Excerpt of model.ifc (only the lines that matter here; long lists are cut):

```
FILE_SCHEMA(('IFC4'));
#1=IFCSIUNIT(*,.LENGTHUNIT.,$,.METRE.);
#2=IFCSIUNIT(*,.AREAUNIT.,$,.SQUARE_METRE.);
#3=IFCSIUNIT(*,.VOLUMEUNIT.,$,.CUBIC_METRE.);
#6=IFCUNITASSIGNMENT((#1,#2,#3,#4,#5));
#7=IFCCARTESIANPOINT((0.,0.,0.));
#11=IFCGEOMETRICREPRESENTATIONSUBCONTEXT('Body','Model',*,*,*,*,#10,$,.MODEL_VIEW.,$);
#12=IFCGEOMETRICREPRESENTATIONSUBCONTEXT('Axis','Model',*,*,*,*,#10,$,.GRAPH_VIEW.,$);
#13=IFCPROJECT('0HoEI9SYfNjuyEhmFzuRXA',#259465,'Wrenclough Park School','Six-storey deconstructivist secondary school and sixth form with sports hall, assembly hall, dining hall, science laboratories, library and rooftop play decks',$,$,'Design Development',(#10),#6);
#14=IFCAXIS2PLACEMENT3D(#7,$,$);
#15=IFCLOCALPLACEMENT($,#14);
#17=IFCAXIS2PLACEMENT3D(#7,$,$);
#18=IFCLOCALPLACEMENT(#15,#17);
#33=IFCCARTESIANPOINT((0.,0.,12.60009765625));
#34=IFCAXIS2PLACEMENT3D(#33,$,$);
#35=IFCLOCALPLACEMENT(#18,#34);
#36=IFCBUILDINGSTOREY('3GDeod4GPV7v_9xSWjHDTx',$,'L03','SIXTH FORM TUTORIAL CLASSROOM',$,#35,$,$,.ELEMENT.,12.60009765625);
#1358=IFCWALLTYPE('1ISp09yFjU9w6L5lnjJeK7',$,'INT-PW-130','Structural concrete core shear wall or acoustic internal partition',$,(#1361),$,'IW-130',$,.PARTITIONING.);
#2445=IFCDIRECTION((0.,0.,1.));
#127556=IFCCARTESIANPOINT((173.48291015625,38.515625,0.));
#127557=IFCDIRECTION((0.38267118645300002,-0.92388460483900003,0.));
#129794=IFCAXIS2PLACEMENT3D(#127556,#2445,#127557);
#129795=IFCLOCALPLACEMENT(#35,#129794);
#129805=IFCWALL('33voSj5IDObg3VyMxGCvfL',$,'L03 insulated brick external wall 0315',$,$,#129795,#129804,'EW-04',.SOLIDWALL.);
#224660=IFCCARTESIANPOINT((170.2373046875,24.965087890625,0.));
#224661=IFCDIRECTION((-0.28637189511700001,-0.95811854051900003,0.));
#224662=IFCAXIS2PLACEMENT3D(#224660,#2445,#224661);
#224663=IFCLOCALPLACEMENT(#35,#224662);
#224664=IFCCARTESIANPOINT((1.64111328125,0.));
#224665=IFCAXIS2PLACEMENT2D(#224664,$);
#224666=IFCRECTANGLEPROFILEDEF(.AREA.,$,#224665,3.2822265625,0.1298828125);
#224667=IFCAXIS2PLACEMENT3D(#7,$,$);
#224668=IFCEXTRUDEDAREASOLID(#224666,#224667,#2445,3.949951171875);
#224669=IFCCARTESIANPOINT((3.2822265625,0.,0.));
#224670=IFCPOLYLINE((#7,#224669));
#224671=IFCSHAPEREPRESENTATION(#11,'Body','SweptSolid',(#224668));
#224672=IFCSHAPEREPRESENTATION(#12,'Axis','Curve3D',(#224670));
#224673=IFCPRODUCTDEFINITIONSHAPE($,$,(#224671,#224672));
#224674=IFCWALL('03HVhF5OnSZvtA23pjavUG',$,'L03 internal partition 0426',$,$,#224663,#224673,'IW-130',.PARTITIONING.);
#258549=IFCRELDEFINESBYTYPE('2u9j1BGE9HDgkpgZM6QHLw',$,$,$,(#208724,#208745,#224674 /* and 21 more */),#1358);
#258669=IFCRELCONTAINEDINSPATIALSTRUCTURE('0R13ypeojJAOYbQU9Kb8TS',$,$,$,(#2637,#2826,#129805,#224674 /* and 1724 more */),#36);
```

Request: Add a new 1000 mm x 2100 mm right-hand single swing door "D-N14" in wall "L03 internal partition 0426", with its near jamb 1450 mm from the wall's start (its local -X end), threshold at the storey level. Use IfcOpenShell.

```python
import numpy as np
import ifcopenshell
import ifcopenshell.api.feature
import ifcopenshell.api.geometry
import ifcopenshell.api.root
import ifcopenshell.api.spatial
import ifcopenshell.geom
import ifcopenshell.util.element
import ifcopenshell.util.placement
import ifcopenshell.util.representation
import ifcopenshell.util.shape
import ifcopenshell.util.unit

model = ifcopenshell.open("model.ifc")
unit_scale = ifcopenshell.util.unit.calculate_unit_scale(model)
settings = ifcopenshell.geom.settings()


def volume(element):
    """Net volume in cubic metres, openings subtracted."""
    shape = ifcopenshell.geom.create_shape(settings, element)
    return ifcopenshell.util.shape.get_volume(shape.geometry)


wall = model.by_guid("03HVhF5OnSZvtA23pjavUG")
storey = ifcopenshell.util.element.get_container(wall, ifc_class="IfcBuildingStorey")
context = ifcopenshell.util.representation.get_context(model, "Model", "Body", "MODEL_VIEW")
before = volume(wall)

width, height, from_end, sill = 1, 2.1, 1.45, 0.0  # metres

# The wall runs along its own X axis, and the end named is its -X end.
wall_shape = ifcopenshell.geom.create_shape(settings, wall)
x, y, z = ifcopenshell.util.shape.get_vertices(wall_shape.geometry).T
start = x.min() + from_end
face, thickness = float(y.min()), float(y.max() - y.min())
wall_matrix = ifcopenshell.util.placement.get_local_placement(wall.ObjectPlacement)
level = ifcopenshell.util.placement.get_local_placement(storey.ObjectPlacement)[2, 3]


def in_wall(x, y):
    """Placement at x, y metres in the wall's axes, at sill height."""
    matrix = wall_matrix.copy()
    matrix[:, 3] = wall_matrix @ np.array([x / unit_scale, y / unit_scale, 0.0, 1.0])
    matrix[2, 3] = level + sill / unit_scale
    return matrix


# Opening: a box that overshoots both wall faces by 50 mm.
opening = ifcopenshell.api.root.create_entity(model, ifc_class="IfcOpeningElement", predefined_type="OPENING")
box = ifcopenshell.api.geometry.add_wall_representation(
    model, context=context, length=width, height=height, thickness=thickness + 0.1
)
ifcopenshell.api.geometry.assign_representation(model, product=opening, representation=box)
ifcopenshell.api.geometry.edit_object_placement(model, product=opening, matrix=in_wall(start, face - 0.05), is_si=False)
ifcopenshell.api.feature.add_feature(model, feature=opening, element=wall)

door = ifcopenshell.api.root.create_entity(model, ifc_class="IfcDoor", name="D-N14", predefined_type="DOOR")
door.OverallWidth, door.OverallHeight = width / unit_scale, height / unit_scale
door.OperationType = "SINGLE_SWING_RIGHT"
body = ifcopenshell.api.geometry.add_door_representation(
    model,
    context=context,
    overall_width=door.OverallWidth,
    overall_height=door.OverallHeight,
    operation_type="SINGLE_SWING_RIGHT",
    lining_properties={"LiningDepth": thickness / unit_scale, "ThresholdDepth": thickness / unit_scale},
)
ifcopenshell.api.geometry.assign_representation(model, product=door, representation=body)
ifcopenshell.api.spatial.assign_container(model, products=[door], relating_structure=storey)
ifcopenshell.api.feature.add_filling(model, opening=opening, element=door)

# The lining spans the wall, so the door starts at the wall face.
ifcopenshell.api.geometry.edit_object_placement(model, product=door, matrix=in_wall(start, face), is_si=False)

after = volume(wall)

print(f"wall volume {before:.3f} -> {after:.3f} m3")

model.write("model_updated.ifc")
```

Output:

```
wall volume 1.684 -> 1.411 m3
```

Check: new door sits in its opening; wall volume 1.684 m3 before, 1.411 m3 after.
